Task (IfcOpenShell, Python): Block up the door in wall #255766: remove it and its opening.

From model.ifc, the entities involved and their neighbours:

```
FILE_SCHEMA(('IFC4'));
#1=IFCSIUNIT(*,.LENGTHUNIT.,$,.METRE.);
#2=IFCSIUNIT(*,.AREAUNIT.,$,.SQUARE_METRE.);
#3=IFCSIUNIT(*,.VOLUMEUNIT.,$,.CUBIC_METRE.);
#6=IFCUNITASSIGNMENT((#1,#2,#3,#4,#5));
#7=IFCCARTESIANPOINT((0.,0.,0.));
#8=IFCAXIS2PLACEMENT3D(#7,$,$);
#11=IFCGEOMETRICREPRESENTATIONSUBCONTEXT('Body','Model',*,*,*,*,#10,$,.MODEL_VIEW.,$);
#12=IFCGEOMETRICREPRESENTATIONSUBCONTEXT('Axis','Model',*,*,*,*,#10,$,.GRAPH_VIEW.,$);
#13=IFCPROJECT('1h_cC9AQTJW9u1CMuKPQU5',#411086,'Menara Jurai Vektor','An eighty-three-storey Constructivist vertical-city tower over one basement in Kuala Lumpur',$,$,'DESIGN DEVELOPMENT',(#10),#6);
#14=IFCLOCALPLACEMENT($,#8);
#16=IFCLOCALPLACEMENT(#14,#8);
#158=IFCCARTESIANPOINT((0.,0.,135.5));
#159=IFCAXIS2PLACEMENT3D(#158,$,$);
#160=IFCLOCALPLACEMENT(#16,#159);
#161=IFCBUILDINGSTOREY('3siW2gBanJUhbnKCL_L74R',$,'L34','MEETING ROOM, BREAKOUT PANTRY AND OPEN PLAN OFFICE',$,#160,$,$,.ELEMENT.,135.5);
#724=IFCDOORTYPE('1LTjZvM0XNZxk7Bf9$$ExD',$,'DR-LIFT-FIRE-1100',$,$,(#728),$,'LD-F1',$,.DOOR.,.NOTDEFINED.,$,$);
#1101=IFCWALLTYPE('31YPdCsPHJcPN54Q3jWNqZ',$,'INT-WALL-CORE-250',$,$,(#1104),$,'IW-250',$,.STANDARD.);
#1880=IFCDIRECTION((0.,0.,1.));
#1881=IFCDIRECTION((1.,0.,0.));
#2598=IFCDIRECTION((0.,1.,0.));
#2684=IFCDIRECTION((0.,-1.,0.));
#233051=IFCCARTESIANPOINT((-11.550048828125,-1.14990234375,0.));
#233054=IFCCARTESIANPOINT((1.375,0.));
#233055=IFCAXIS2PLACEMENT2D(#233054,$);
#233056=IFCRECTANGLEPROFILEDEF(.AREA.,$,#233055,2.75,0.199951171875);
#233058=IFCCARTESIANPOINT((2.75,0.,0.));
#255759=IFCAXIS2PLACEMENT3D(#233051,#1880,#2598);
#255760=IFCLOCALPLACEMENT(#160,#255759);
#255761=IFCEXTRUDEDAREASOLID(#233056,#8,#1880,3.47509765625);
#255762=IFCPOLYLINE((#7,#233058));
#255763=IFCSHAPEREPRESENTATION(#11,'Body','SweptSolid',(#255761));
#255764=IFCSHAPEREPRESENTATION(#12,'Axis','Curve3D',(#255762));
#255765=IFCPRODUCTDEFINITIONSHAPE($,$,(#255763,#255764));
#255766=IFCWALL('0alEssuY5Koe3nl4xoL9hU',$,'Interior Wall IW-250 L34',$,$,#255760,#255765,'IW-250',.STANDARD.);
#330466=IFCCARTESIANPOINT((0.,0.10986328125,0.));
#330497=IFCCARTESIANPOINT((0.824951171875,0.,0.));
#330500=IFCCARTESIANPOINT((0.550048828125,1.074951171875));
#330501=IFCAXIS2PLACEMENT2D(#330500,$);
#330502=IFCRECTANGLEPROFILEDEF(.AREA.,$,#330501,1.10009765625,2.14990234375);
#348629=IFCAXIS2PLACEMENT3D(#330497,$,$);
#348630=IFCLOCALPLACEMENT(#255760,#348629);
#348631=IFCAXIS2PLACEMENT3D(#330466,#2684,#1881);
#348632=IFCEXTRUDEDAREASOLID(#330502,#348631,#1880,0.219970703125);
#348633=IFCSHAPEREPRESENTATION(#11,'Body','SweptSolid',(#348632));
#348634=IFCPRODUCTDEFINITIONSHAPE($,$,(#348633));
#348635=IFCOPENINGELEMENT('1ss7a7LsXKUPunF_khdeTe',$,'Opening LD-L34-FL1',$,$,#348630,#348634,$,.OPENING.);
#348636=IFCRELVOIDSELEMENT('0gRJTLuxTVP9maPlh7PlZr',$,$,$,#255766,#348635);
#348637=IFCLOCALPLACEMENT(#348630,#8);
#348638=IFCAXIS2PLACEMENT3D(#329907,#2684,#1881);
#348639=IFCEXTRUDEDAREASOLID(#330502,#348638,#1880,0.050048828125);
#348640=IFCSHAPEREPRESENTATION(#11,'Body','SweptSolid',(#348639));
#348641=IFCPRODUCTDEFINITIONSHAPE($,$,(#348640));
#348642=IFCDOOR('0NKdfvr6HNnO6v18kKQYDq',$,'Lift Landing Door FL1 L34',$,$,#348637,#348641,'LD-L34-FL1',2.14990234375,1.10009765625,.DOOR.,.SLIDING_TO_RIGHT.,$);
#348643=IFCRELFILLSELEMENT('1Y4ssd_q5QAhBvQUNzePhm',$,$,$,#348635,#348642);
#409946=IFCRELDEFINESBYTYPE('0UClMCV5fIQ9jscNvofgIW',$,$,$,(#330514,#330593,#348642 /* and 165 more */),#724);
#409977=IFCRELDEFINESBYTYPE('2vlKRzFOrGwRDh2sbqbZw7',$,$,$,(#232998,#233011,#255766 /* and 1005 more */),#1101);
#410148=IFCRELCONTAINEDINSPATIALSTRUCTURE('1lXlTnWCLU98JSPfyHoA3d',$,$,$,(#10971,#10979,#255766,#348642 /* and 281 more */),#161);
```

```python
import ifcopenshell
import ifcopenshell.api.feature
import ifcopenshell.api.root
import ifcopenshell.geom
import ifcopenshell.util.shape

model = ifcopenshell.open("model.ifc")
settings = ifcopenshell.geom.settings()


def volume(element):
    """Net volume in cubic metres, openings subtracted."""
    shape = ifcopenshell.geom.create_shape(settings, element)
    return ifcopenshell.util.shape.get_volume(shape.geometry)


door = model.by_guid("0NKdfvr6HNnO6v18kKQYDq")
opening = door.FillsVoids[0].RelatingOpeningElement
wall = opening.VoidsElements[0].RelatingBuildingElement
before = volume(wall)

ifcopenshell.api.root.remove_product(model, product=door)
ifcopenshell.api.feature.remove_feature(model, feature=opening)

after = volume(wall)

print(f"wall volume {before:.3f} -> {after:.3f} m3")

model.write("model_edited.ifc")
```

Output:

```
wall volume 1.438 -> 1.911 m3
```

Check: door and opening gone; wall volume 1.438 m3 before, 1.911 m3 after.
